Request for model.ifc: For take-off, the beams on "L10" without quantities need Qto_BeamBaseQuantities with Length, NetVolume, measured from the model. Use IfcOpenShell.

First a look at what the model holds.

```python
import ifcopenshell
import ifcopenshell.util.element
import ifcopenshell.util.unit

model = ifcopenshell.open("model.ifc")
print(model.schema)
for unit_type in ("LENGTHUNIT", "AREAUNIT", "VOLUMEUNIT"):
    print(unit_type, ifcopenshell.util.unit.calculate_unit_scale(model, unit_type))
storey = next(s for s in model.by_type("IfcBuildingStorey") if s.Name == "L10")
beams = [e for e in ifcopenshell.util.element.get_decomposition(storey) if e.is_a("IfcBeam")]
for e in sorted(beams, key=lambda e: e.id()):
    print(e.id(), e.is_a(), e.Name, list(ifcopenshell.util.element.get_psets(e, qtos_only=True)), sep=" | ")
```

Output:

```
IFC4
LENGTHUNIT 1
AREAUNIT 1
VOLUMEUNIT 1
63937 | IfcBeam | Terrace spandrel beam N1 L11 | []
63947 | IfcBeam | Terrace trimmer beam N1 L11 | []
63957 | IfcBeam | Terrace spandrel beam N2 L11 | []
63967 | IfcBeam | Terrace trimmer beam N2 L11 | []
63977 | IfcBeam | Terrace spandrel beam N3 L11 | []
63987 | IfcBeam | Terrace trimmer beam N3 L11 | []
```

```python
import ifcopenshell
import ifcopenshell.api.pset
import ifcopenshell.geom
import ifcopenshell.util.element
import ifcopenshell.util.shape
import ifcopenshell.util.unit

model = ifcopenshell.open("model.ifc")
unit_scale = ifcopenshell.util.unit.calculate_unit_scale(model)
volume_scale = ifcopenshell.util.unit.calculate_unit_scale(model, "VOLUMEUNIT")
settings = ifcopenshell.geom.settings()

storey = next(s for s in model.by_type("IfcBuildingStorey") if s.Name == "L10")
beams = [e for e in ifcopenshell.util.element.get_decomposition(storey) if e.is_a("IfcBeam")]

for e in sorted(beams, key=lambda e: e.id()):
    if ifcopenshell.util.element.get_psets(e, qtos_only=True, should_inherit=False):
        continue
    # Geometry comes back in metres, in the element's own axes.
    shape = ifcopenshell.geom.create_shape(settings, e)
    values = {
        "Length": ifcopenshell.util.shape.get_max_xyz(shape.geometry) / unit_scale,
        "NetVolume": ifcopenshell.util.shape.get_volume(shape.geometry) / volume_scale,
    }
    qto = ifcopenshell.api.pset.add_qto(model, product=e, name="Qto_BeamBaseQuantities")
    ifcopenshell.api.pset.edit_qto(model, qto=qto, properties=values)
    print(e.id(), {k: round(v, 3) for k, v in values.items()})

model.write("model_v2.ifc")
```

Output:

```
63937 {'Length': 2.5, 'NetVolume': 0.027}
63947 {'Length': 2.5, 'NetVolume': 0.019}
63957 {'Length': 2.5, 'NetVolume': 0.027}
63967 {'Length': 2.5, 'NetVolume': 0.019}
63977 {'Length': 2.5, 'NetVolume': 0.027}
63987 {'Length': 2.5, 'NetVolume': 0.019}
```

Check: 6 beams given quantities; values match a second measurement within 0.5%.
